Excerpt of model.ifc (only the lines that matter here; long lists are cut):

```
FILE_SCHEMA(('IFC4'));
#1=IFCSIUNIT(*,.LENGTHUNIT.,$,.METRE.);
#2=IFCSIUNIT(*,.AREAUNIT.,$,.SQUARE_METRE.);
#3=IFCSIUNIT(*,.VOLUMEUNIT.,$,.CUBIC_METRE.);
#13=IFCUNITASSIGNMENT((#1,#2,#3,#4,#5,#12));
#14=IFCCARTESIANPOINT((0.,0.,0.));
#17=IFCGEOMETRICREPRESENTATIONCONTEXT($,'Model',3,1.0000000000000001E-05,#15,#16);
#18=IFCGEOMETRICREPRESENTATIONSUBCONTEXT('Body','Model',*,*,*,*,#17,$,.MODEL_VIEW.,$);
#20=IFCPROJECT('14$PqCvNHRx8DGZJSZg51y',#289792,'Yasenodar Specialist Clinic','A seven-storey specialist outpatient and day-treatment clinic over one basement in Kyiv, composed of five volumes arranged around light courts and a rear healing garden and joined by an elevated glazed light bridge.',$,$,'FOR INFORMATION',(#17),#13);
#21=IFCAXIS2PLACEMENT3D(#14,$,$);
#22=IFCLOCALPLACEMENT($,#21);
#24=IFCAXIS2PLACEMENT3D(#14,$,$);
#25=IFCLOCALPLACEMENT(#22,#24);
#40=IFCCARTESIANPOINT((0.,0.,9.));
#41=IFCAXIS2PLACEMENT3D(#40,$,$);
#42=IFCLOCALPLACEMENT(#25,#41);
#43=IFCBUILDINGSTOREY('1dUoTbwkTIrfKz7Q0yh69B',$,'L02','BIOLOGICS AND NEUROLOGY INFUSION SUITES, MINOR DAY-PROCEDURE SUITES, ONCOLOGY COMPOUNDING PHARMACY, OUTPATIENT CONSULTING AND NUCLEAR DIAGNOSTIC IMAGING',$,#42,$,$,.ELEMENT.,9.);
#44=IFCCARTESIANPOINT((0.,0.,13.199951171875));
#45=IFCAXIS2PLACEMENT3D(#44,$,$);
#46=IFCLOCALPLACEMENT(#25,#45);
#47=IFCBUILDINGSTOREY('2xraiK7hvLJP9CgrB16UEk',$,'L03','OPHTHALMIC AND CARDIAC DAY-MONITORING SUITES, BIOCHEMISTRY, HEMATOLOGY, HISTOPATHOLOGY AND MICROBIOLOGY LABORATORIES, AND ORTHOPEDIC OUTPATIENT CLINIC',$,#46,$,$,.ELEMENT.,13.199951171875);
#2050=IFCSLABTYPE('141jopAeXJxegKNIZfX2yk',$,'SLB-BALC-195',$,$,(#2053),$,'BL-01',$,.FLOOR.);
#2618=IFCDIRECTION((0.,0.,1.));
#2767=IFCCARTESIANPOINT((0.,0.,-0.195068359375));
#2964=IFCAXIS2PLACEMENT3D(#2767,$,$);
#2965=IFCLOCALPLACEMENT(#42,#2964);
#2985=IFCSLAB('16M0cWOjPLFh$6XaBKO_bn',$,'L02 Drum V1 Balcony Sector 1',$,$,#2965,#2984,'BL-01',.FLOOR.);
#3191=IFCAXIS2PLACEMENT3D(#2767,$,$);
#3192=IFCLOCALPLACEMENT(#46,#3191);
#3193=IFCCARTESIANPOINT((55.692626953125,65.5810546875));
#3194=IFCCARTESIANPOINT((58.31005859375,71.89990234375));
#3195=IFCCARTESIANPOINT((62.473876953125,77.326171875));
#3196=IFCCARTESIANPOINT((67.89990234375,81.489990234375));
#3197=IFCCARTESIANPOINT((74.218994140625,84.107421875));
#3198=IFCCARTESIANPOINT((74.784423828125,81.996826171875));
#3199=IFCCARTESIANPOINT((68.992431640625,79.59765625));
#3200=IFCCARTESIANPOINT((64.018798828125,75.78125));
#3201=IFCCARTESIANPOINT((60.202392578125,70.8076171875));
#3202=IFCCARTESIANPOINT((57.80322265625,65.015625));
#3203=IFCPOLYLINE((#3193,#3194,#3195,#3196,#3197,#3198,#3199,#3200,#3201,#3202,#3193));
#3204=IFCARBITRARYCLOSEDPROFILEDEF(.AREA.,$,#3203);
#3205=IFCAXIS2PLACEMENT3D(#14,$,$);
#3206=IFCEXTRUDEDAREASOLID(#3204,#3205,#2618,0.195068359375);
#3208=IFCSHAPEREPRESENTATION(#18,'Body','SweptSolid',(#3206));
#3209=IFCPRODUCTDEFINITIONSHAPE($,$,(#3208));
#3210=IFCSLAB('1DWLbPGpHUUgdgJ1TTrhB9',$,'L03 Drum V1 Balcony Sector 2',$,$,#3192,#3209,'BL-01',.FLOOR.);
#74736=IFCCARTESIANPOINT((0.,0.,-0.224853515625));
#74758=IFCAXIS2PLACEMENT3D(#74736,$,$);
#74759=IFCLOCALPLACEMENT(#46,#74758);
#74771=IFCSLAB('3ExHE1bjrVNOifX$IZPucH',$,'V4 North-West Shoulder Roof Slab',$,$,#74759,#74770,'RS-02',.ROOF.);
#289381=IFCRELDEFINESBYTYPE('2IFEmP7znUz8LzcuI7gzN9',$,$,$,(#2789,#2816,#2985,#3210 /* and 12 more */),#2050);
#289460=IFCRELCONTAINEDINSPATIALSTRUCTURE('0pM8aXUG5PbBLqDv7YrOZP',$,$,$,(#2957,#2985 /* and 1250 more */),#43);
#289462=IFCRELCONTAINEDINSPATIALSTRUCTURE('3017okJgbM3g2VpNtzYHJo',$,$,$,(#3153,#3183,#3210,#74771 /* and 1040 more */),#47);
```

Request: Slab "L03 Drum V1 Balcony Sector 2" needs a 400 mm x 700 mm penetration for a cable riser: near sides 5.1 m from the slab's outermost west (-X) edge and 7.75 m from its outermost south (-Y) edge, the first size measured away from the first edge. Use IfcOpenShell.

```python
import numpy as np
import ifcopenshell
import ifcopenshell.api.feature
import ifcopenshell.api.geometry
import ifcopenshell.api.root
import ifcopenshell.geom
import ifcopenshell.util.placement
import ifcopenshell.util.representation
import ifcopenshell.util.shape
import ifcopenshell.util.unit

model = ifcopenshell.open("model.ifc")
unit_scale = ifcopenshell.util.unit.calculate_unit_scale(model)
settings = ifcopenshell.geom.settings()


def volume(element):
    """Net volume in cubic metres, openings subtracted."""
    shape = ifcopenshell.geom.create_shape(settings, element)
    return ifcopenshell.util.shape.get_volume(shape.geometry)


slab = model.by_guid("1DWLbPGpHUUgdgJ1TTrhB9")
before = volume(slab)

# Extent in the slab's own axes, in metres. The edges named are its -X and -Y sides.
slab_shape = ifcopenshell.geom.create_shape(settings, slab)
vertices = ifcopenshell.util.shape.get_vertices(slab_shape.geometry)
x_min, y_min, bottom = vertices.min(axis=0)
top = vertices[:, 2].max()

opening = ifcopenshell.api.root.create_entity(model, ifc_class="IfcOpeningElement", name="Cable riser opening", predefined_type="OPENING")
context = ifcopenshell.util.representation.get_context(model, "Model", "Body", "MODEL_VIEW")
width, depth = 0.4, 0.7
outline = [(0.0, 0.0), (width, 0.0), (width, depth), (0.0, depth), (0.0, 0.0)]
# Overshoot both faces by 50 mm so the cut is clean.
shape = ifcopenshell.api.geometry.add_slab_representation(
    model, context=context, depth=top - bottom + 0.1, polyline=outline
)
ifcopenshell.api.geometry.assign_representation(model, product=opening, representation=shape)

matrix = ifcopenshell.util.placement.get_local_placement(slab.ObjectPlacement)
matrix[:, 3] = matrix @ np.append(np.array([x_min + 5.1, y_min + 7.75, bottom - 0.05]) / unit_scale, 1.0)
ifcopenshell.api.geometry.edit_object_placement(model, product=opening, matrix=matrix, is_si=False)
ifcopenshell.api.feature.add_feature(model, feature=opening, element=slab)

after = volume(slab)

print(f"slab volume {before:.3f} -> {after:.3f} m3")

model.write("model_rev.ifc")
```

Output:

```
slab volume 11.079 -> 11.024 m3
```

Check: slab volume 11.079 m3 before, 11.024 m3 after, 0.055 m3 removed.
